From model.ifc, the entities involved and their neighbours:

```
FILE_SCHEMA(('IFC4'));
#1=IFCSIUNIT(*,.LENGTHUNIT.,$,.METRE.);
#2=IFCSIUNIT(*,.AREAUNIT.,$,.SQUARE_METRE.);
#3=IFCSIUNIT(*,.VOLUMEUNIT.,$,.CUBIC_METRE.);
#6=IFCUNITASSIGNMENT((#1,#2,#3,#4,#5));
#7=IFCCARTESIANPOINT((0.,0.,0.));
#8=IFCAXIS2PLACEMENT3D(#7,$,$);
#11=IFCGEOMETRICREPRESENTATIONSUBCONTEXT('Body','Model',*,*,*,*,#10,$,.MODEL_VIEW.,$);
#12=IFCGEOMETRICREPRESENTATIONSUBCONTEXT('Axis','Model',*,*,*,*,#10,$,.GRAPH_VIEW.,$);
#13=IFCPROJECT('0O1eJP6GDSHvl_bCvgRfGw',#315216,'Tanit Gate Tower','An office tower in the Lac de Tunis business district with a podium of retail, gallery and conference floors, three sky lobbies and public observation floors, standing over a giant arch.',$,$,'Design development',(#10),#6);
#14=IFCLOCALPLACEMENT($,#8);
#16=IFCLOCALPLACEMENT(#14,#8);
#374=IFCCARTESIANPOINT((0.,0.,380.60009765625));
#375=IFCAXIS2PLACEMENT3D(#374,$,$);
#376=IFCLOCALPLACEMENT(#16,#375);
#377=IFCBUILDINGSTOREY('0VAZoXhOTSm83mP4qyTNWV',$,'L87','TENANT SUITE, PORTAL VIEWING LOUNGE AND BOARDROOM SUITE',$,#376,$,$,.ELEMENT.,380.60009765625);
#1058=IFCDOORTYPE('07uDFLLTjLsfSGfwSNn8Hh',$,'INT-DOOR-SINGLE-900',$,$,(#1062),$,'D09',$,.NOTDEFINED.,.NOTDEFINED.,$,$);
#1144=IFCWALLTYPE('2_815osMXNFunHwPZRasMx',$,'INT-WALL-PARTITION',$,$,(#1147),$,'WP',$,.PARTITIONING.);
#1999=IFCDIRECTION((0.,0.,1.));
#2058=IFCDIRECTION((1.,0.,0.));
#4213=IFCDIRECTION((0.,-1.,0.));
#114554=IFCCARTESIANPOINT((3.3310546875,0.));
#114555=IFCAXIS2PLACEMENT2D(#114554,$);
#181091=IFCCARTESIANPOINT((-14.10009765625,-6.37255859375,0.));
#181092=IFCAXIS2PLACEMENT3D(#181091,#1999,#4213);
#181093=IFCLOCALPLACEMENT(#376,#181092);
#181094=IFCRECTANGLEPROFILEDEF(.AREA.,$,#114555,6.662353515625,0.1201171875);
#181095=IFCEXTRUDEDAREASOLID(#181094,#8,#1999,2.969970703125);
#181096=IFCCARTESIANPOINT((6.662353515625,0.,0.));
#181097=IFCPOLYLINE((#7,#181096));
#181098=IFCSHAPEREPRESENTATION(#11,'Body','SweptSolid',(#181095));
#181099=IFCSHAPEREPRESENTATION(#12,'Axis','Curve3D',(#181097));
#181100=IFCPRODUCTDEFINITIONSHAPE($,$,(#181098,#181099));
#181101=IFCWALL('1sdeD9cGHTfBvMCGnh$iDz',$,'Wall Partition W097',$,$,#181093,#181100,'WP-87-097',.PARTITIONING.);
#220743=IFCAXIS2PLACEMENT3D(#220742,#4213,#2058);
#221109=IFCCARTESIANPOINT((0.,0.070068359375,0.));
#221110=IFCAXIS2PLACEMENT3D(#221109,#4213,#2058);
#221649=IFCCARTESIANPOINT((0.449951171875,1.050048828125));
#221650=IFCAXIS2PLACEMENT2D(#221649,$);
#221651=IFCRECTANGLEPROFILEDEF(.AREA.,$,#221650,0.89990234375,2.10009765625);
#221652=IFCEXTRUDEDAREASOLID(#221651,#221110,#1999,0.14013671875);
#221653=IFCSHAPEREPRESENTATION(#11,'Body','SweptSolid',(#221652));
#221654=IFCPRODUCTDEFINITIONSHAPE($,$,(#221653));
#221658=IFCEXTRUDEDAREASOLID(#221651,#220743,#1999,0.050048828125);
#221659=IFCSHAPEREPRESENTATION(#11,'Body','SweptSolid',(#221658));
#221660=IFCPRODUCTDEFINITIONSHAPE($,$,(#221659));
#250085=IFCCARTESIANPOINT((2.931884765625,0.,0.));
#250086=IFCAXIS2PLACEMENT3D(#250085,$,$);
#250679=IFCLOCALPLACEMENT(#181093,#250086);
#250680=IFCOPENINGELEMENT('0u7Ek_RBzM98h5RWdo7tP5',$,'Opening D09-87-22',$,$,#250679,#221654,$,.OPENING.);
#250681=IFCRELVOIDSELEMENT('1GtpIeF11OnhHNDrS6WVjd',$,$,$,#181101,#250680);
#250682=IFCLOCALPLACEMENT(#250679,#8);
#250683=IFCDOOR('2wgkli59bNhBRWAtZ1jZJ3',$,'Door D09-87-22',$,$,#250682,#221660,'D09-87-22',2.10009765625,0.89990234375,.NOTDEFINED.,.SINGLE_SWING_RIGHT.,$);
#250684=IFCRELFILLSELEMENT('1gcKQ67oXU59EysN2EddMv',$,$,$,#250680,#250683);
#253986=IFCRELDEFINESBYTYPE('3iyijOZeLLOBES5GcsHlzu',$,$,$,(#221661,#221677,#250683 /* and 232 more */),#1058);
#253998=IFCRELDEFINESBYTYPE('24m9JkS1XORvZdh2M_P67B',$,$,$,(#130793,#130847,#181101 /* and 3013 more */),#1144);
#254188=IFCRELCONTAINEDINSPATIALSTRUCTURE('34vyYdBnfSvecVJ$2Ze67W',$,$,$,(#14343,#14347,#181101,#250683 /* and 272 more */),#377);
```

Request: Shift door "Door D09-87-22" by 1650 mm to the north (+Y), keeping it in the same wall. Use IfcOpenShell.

```python
import ifcopenshell
import ifcopenshell.api.geometry
import ifcopenshell.util.placement
import ifcopenshell.util.unit

model = ifcopenshell.open("model.ifc")
unit_scale = ifcopenshell.util.unit.calculate_unit_scale(model)

door = model.by_guid("2wgkli59bNhBRWAtZ1jZJ3")
opening = door.FillsVoids[0].RelatingOpeningElement
wall = opening.VoidsElements[0].RelatingBuildingElement

wall_matrix = ifcopenshell.util.placement.get_local_placement(wall.ObjectPlacement)
shift = wall_matrix[:3, 0] * -1.65 / unit_scale
before = ifcopenshell.util.placement.get_local_placement(door.ObjectPlacement)[:3, 3].copy()

# The door is placed relative to its opening, so it follows when the opening moves.
matrix = ifcopenshell.util.placement.get_local_placement(opening.ObjectPlacement)
matrix[:3, 3] += shift
ifcopenshell.api.geometry.edit_object_placement(
    model, product=opening, matrix=matrix, is_si=False, should_transform_children=True
)

after = ifcopenshell.util.placement.get_local_placement(door.ObjectPlacement)[:3, 3]
print("door moved by", (after - before).round(3) + 0.0)

model.write("model_v2.ifc")
```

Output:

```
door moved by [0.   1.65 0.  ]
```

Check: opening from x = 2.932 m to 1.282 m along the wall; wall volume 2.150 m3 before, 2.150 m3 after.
